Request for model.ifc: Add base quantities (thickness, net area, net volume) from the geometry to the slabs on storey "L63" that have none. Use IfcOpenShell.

First a look at what the model holds.

```python
import ifcopenshell
import ifcopenshell.util.element
import ifcopenshell.util.unit

model = ifcopenshell.open("model.ifc")
print(model.schema)
for unit_type in ("LENGTHUNIT", "AREAUNIT", "VOLUMEUNIT"):
    print(unit_type, ifcopenshell.util.unit.calculate_unit_scale(model, unit_type))
storey = next(s for s in model.by_type("IfcBuildingStorey") if s.Name == "L63")
slabs = [e for e in ifcopenshell.util.element.get_decomposition(storey) if e.is_a("IfcSlab")]
for e in sorted(slabs, key=lambda e: e.id()):
    print(e.id(), e.is_a(), e.Name, list(ifcopenshell.util.element.get_psets(e, qtos_only=True)), sep=" | ")
```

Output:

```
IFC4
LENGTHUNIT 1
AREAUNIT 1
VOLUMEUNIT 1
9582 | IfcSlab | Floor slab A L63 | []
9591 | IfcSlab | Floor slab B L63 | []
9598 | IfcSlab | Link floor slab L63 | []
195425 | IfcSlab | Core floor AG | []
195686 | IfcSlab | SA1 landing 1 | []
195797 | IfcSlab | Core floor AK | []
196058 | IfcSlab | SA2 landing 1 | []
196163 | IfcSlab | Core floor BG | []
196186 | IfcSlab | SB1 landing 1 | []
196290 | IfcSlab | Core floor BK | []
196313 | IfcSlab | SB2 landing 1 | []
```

```python
import ifcopenshell
import ifcopenshell.api.pset
import ifcopenshell.geom
import ifcopenshell.util.element
import ifcopenshell.util.shape
import ifcopenshell.util.unit

model = ifcopenshell.open("model.ifc")
unit_scale = ifcopenshell.util.unit.calculate_unit_scale(model)
area_scale = ifcopenshell.util.unit.calculate_unit_scale(model, "AREAUNIT")
volume_scale = ifcopenshell.util.unit.calculate_unit_scale(model, "VOLUMEUNIT")
settings = ifcopenshell.geom.settings()

storey = next(s for s in model.by_type("IfcBuildingStorey") if s.Name == "L63")
slabs = [e for e in ifcopenshell.util.element.get_decomposition(storey) if e.is_a("IfcSlab")]

for e in sorted(slabs, key=lambda e: e.id()):
    if ifcopenshell.util.element.get_psets(e, qtos_only=True, should_inherit=False):
        continue
    # Geometry comes back in metres, in the element's own axes.
    shape = ifcopenshell.geom.create_shape(settings, e)
    values = {
        "Width": ifcopenshell.util.shape.get_z(shape.geometry) / unit_scale,
        "NetArea": ifcopenshell.util.shape.get_footprint_area(shape.geometry) / area_scale,
        "NetVolume": ifcopenshell.util.shape.get_volume(shape.geometry) / volume_scale,
    }
    qto = ifcopenshell.api.pset.add_qto(model, product=e, name="Qto_SlabBaseQuantities")
    ifcopenshell.api.pset.edit_qto(model, qto=qto, properties=values)
    print(e.id(), {k: round(v, 3) for k, v in values.items()})

model.write("model_edited.ifc")
```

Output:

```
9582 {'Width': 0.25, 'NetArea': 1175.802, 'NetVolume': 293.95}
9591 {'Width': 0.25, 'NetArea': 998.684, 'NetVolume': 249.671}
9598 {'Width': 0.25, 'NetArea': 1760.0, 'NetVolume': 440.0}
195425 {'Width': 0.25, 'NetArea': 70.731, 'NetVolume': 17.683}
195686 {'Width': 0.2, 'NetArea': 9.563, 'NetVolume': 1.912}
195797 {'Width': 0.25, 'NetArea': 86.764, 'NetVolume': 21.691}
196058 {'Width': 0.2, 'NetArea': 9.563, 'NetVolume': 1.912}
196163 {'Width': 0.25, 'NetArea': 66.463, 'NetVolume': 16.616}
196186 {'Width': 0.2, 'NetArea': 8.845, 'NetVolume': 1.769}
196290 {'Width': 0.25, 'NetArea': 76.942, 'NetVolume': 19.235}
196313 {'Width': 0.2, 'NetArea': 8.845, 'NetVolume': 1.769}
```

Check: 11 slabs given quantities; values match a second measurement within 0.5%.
